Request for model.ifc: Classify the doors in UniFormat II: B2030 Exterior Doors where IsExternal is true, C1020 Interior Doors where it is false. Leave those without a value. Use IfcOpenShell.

First a look at what the model holds.

```python
import ifcopenshell
import ifcopenshell.util.element

model = ifcopenshell.open("model.ifc")
print(model.schema)
print("classifications:", [c.Name for c in model.by_type("IfcClassification")])
values = [ifcopenshell.util.element.get_pset(e, "Pset_DoorCommon", "IsExternal") for e in model.by_type("IfcDoor")]
for value in (True, False, None):
    print("IsExternal", value, values.count(value))
```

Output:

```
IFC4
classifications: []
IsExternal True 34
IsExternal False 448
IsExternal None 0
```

```python
import ifcopenshell
import ifcopenshell.api.classification
import ifcopenshell.util.element

model = ifcopenshell.open("model.ifc")

system = ifcopenshell.api.classification.add_classification(model, classification="UniFormat II")

doors = model.by_type("IfcDoor")
external = {e: ifcopenshell.util.element.get_pset(e, "Pset_DoorCommon", "IsExternal") for e in doors}
for flag, code, name in ((True, "B2030", "Exterior Doors"), (False, "C1020", "Interior Doors")):
    products = [e for e in doors if external[e] is flag]
    ifcopenshell.api.classification.add_reference(
        model, products=products, classification=system, identification=code, name=name
    )
    print(code, len(products))

model.write("model_v2.ifc")
```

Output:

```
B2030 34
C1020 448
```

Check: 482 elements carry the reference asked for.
